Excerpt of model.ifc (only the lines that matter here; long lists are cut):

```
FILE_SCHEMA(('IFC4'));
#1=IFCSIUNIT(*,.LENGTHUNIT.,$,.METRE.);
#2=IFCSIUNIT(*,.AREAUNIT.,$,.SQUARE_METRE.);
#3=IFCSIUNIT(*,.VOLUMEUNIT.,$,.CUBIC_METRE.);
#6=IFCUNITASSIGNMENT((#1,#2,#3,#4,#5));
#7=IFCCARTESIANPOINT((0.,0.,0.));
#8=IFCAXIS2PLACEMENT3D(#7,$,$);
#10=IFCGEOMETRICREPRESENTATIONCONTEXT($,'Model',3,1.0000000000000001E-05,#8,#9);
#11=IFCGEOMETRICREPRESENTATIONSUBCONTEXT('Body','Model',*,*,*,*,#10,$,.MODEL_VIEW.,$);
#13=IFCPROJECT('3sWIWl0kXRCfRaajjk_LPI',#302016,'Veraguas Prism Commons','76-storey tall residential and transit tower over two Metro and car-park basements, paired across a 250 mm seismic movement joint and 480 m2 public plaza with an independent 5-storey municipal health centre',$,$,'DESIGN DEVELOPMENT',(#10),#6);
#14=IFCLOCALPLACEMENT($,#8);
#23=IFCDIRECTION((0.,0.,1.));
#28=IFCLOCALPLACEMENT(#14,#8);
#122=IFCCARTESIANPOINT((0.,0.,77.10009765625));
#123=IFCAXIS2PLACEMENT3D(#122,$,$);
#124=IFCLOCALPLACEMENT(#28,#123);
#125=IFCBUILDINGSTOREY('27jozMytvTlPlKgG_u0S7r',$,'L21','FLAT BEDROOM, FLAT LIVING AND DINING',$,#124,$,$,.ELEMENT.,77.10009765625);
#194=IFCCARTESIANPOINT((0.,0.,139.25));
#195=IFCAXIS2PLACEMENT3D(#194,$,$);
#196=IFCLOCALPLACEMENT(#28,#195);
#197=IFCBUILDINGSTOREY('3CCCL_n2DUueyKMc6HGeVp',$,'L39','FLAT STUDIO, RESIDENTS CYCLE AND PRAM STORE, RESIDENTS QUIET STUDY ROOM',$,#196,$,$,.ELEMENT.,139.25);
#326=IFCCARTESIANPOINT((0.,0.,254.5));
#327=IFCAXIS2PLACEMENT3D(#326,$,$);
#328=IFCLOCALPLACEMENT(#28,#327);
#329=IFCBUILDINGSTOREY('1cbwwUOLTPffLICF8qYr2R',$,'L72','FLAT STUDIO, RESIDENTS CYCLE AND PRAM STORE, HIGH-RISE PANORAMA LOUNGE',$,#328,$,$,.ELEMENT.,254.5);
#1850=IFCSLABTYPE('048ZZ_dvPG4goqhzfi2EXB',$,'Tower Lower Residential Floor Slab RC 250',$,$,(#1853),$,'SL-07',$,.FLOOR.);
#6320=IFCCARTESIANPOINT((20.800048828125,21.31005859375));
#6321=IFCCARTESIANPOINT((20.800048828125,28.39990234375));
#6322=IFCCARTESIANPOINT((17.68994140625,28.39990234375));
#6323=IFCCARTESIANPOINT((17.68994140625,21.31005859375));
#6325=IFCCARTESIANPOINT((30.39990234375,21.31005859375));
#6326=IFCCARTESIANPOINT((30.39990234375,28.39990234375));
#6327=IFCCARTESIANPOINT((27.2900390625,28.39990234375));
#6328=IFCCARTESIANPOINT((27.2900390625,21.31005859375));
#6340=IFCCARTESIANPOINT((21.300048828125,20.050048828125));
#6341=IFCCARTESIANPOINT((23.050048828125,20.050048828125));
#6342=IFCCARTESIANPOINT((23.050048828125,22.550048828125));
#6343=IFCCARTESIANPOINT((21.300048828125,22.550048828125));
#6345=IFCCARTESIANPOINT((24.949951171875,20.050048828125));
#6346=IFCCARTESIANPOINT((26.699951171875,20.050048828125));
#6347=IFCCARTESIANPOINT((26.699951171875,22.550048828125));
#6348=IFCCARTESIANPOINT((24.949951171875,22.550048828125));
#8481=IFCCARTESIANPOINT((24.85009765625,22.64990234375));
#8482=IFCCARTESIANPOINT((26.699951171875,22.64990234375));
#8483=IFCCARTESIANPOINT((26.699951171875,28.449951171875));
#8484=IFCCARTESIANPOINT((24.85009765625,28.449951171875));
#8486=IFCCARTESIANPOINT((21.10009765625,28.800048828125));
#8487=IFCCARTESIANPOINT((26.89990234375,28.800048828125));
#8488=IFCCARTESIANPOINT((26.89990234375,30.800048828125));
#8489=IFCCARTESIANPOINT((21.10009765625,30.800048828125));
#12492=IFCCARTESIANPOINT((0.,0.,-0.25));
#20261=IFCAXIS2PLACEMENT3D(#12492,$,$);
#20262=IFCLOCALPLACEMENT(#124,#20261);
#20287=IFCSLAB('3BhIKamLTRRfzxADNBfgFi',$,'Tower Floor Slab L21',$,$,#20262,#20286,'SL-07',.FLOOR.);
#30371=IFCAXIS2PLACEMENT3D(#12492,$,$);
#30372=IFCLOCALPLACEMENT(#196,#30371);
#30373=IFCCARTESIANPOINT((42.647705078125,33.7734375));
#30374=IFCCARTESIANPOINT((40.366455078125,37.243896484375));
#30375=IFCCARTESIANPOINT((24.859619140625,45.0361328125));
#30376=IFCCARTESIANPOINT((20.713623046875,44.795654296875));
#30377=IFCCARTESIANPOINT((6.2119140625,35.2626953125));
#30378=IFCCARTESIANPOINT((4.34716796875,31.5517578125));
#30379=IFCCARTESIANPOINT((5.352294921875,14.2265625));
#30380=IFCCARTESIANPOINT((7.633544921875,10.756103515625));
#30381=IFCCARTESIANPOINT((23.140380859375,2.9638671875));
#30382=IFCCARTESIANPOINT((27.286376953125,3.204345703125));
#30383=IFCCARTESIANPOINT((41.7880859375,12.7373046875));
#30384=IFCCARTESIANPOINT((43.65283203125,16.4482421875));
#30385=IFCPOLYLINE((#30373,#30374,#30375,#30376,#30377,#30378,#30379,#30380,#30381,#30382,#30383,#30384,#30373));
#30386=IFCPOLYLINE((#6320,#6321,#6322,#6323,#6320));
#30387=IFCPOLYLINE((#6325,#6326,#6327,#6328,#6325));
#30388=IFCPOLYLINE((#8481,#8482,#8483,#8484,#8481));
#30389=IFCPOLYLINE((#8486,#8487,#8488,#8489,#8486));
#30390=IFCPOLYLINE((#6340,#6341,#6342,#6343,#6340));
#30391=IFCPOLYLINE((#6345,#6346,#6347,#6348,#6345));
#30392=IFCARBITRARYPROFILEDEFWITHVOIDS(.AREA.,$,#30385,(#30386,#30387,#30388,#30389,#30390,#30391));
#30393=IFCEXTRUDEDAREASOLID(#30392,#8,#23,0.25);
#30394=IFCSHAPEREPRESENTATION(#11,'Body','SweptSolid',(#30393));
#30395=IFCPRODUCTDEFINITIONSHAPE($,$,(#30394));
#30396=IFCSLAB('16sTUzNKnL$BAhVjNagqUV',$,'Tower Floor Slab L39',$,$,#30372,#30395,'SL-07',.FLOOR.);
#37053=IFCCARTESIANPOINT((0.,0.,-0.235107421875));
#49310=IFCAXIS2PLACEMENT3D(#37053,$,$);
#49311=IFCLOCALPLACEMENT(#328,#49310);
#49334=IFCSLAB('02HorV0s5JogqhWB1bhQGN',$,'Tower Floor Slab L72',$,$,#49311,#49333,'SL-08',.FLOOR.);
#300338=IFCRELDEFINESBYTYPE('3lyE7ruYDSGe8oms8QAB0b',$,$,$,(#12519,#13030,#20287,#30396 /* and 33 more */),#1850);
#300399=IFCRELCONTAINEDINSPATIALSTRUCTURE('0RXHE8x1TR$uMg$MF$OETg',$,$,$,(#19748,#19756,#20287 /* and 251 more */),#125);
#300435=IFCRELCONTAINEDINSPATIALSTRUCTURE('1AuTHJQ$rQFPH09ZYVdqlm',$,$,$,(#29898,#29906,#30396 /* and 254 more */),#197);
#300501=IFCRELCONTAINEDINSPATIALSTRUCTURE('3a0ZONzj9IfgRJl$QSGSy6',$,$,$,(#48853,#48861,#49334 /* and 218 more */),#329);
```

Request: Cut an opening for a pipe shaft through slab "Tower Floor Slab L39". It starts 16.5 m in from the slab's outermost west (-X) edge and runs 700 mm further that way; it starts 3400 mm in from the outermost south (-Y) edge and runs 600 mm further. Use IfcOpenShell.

```python
import numpy as np
import ifcopenshell
import ifcopenshell.api.feature
import ifcopenshell.api.geometry
import ifcopenshell.api.root
import ifcopenshell.geom
import ifcopenshell.util.placement
import ifcopenshell.util.representation
import ifcopenshell.util.shape
import ifcopenshell.util.unit

model = ifcopenshell.open("model.ifc")
unit_scale = ifcopenshell.util.unit.calculate_unit_scale(model)
settings = ifcopenshell.geom.settings()


def volume(element):
    """Net volume in cubic metres, openings subtracted."""
    shape = ifcopenshell.geom.create_shape(settings, element)
    return ifcopenshell.util.shape.get_volume(shape.geometry)


slab = model.by_guid("16sTUzNKnL$BAhVjNagqUV")
before = volume(slab)

# Extent in the slab's own axes, in metres. The edges named are its -X and -Y sides.
slab_shape = ifcopenshell.geom.create_shape(settings, slab)
vertices = ifcopenshell.util.shape.get_vertices(slab_shape.geometry)
x_min, y_min, bottom = vertices.min(axis=0)
top = vertices[:, 2].max()

opening = ifcopenshell.api.root.create_entity(model, ifc_class="IfcOpeningElement", name="Pipe shaft opening", predefined_type="OPENING")
context = ifcopenshell.util.representation.get_context(model, "Model", "Body", "MODEL_VIEW")
width, depth = 0.7, 0.6
outline = [(0.0, 0.0), (width, 0.0), (width, depth), (0.0, depth), (0.0, 0.0)]
# Overshoot both faces by 50 mm so the cut is clean.
shape = ifcopenshell.api.geometry.add_slab_representation(
    model, context=context, depth=top - bottom + 0.1, polyline=outline
)
ifcopenshell.api.geometry.assign_representation(model, product=opening, representation=shape)

matrix = ifcopenshell.util.placement.get_local_placement(slab.ObjectPlacement)
matrix[:, 3] = matrix @ np.append(np.array([x_min + 16.5, y_min + 3.4, bottom - 0.05]) / unit_scale, 1.0)
ifcopenshell.api.geometry.edit_object_placement(model, product=opening, matrix=matrix, is_si=False)
ifcopenshell.api.feature.add_feature(model, feature=opening, element=slab)

after = volume(slab)

print(f"slab volume {before:.3f} -> {after:.3f} m3")

model.write("model_edited.ifc")
```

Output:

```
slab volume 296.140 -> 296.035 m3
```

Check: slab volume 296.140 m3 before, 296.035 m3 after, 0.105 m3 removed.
